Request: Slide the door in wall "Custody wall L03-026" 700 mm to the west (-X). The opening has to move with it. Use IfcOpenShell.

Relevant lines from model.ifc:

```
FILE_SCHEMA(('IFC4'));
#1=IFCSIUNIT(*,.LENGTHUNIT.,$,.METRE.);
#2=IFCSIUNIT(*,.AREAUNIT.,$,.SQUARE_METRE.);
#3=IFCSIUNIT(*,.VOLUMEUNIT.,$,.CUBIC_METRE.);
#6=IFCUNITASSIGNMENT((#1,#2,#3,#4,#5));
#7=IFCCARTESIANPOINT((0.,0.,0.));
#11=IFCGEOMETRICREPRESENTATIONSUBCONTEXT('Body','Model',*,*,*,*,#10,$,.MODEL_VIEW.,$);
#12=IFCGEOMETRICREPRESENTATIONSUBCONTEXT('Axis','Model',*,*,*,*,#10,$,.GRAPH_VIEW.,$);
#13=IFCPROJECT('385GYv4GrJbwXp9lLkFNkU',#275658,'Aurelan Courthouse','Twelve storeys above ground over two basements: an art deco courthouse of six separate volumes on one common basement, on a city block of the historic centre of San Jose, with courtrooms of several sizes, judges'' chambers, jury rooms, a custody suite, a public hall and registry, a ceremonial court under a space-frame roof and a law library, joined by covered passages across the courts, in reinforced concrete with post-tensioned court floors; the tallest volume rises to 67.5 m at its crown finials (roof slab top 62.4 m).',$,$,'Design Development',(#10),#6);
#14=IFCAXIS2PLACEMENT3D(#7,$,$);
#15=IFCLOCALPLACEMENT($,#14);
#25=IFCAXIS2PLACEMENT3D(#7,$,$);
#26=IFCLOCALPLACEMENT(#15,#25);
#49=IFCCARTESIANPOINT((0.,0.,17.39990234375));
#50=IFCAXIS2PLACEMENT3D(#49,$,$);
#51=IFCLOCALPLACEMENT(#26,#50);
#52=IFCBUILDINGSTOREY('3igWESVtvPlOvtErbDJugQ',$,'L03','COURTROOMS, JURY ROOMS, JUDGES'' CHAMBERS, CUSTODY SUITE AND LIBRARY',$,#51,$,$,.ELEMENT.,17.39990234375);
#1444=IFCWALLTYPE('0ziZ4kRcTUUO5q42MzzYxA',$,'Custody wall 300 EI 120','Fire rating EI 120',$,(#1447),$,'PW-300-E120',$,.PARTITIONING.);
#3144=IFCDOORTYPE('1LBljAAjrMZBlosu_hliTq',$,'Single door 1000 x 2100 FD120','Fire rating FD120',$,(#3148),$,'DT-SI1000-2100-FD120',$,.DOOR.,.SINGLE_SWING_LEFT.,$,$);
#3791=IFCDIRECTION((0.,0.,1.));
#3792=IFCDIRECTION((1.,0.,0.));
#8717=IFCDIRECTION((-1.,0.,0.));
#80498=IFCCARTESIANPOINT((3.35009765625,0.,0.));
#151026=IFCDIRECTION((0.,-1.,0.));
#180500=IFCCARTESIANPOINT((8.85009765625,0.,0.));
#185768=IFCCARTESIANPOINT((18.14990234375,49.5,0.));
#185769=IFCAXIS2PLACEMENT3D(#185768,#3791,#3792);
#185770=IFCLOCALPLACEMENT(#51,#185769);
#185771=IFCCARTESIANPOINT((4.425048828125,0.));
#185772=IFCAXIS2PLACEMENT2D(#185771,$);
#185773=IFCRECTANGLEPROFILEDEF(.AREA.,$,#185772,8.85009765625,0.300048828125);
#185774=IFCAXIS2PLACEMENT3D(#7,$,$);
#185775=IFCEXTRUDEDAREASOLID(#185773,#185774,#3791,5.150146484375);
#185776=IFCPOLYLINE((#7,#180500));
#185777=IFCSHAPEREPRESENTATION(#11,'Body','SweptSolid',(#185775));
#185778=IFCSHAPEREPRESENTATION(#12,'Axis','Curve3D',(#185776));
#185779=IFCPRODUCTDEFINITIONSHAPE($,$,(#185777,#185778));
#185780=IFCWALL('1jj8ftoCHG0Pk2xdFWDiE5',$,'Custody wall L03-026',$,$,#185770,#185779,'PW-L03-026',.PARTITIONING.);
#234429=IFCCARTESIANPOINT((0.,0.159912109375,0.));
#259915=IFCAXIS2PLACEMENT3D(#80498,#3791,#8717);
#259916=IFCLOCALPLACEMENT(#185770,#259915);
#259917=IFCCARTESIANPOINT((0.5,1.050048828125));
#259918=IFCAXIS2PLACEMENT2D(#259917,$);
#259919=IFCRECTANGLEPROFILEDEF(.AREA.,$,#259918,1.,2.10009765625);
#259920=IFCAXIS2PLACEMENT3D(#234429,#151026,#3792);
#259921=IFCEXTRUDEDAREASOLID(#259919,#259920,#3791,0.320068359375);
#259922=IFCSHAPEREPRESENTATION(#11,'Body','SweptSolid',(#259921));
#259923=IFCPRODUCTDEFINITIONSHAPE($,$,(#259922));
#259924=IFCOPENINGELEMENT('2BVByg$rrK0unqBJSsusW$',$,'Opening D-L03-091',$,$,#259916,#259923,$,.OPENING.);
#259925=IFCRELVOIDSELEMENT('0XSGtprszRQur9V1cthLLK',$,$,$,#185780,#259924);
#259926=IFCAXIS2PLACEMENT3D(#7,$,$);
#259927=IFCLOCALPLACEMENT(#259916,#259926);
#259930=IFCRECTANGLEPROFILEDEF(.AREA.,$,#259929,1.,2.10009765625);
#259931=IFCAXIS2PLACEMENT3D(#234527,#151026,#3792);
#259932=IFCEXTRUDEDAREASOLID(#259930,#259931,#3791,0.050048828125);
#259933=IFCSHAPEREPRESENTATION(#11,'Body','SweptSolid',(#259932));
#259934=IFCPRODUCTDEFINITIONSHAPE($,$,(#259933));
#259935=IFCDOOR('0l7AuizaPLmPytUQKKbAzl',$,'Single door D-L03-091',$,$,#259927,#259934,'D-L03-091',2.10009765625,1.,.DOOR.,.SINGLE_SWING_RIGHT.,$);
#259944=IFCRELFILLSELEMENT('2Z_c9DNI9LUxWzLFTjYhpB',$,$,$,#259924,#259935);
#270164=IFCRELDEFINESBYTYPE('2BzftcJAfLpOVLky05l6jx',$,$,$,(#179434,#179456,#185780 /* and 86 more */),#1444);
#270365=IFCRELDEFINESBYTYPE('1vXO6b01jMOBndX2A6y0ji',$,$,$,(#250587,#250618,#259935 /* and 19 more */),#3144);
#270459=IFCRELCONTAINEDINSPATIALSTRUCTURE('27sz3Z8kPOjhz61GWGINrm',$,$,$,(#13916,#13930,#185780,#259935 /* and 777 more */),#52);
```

```python
import ifcopenshell
import ifcopenshell.api.geometry
import ifcopenshell.util.placement
import ifcopenshell.util.unit

model = ifcopenshell.open("model.ifc")
unit_scale = ifcopenshell.util.unit.calculate_unit_scale(model)

door = model.by_guid("0l7AuizaPLmPytUQKKbAzl")
opening = door.FillsVoids[0].RelatingOpeningElement
wall = opening.VoidsElements[0].RelatingBuildingElement

wall_matrix = ifcopenshell.util.placement.get_local_placement(wall.ObjectPlacement)
shift = wall_matrix[:3, 0] * -0.7 / unit_scale
before = ifcopenshell.util.placement.get_local_placement(door.ObjectPlacement)[:3, 3].copy()

# The door is placed relative to its opening, so it follows when the opening moves.
matrix = ifcopenshell.util.placement.get_local_placement(opening.ObjectPlacement)
matrix[:3, 3] += shift
ifcopenshell.api.geometry.edit_object_placement(
    model, product=opening, matrix=matrix, is_si=False, should_transform_children=True
)

after = ifcopenshell.util.placement.get_local_placement(door.ObjectPlacement)[:3, 3]
print("door moved by", (after - before).round(3) + 0.0)

model.write("model_v2.ifc")
```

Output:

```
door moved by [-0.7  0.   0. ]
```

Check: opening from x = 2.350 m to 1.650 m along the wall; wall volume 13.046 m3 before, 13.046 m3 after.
